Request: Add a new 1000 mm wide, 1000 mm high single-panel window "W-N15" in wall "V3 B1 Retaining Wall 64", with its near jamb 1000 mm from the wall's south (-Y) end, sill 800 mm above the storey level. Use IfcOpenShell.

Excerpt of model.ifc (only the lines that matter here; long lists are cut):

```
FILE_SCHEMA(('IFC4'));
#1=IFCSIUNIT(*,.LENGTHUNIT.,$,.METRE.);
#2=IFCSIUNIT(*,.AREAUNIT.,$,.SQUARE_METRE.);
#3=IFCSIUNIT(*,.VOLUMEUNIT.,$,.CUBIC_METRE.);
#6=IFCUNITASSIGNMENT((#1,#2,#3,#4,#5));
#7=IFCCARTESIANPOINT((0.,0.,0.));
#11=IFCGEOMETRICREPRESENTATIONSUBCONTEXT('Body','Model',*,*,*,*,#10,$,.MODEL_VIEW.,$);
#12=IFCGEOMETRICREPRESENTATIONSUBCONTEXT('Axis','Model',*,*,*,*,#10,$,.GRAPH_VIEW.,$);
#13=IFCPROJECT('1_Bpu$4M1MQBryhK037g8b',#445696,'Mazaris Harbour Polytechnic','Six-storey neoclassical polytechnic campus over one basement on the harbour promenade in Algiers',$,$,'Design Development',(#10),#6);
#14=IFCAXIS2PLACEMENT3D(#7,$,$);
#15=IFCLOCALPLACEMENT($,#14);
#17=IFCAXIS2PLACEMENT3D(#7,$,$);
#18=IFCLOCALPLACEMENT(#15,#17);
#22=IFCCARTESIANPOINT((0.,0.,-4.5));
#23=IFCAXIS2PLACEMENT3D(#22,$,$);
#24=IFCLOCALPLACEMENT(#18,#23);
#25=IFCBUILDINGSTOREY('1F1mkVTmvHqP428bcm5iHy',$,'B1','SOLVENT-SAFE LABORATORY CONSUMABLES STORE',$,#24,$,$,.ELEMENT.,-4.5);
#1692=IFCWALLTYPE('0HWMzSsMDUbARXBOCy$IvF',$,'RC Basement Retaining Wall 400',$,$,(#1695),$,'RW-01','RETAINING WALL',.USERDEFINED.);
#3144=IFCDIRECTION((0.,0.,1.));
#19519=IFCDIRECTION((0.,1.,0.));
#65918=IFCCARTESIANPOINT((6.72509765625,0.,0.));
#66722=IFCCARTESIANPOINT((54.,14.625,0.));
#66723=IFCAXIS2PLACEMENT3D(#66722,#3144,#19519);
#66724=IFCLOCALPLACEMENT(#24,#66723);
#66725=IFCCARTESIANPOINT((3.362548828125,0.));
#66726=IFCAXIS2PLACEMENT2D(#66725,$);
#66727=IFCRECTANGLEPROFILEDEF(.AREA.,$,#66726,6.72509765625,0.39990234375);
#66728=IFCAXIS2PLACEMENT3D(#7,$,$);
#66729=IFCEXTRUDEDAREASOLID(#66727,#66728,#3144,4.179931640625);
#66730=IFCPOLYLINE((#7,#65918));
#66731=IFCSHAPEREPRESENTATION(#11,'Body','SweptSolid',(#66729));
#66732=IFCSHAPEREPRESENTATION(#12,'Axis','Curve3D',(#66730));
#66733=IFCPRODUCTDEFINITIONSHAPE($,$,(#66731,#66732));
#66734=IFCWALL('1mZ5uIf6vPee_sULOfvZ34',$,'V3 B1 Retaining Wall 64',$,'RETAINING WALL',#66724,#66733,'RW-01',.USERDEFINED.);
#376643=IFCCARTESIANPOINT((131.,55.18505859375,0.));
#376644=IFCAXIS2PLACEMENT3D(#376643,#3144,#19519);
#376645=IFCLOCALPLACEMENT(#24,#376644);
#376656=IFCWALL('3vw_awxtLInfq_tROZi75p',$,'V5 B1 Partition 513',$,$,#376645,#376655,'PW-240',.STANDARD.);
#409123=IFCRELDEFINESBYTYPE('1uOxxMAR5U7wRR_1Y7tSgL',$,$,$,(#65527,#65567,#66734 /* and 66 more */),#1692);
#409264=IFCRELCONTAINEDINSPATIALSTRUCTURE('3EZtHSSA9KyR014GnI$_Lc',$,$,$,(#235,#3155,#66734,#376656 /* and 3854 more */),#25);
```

```python
import numpy as np
import ifcopenshell
import ifcopenshell.api.feature
import ifcopenshell.api.geometry
import ifcopenshell.api.root
import ifcopenshell.api.spatial
import ifcopenshell.geom
import ifcopenshell.util.element
import ifcopenshell.util.placement
import ifcopenshell.util.representation
import ifcopenshell.util.shape
import ifcopenshell.util.unit

model = ifcopenshell.open("model.ifc")
unit_scale = ifcopenshell.util.unit.calculate_unit_scale(model)
settings = ifcopenshell.geom.settings()


def volume(element):
    """Net volume in cubic metres, openings subtracted."""
    shape = ifcopenshell.geom.create_shape(settings, element)
    return ifcopenshell.util.shape.get_volume(shape.geometry)


wall = model.by_guid("1mZ5uIf6vPee_sULOfvZ34")
storey = ifcopenshell.util.element.get_container(wall, ifc_class="IfcBuildingStorey")
context = ifcopenshell.util.representation.get_context(model, "Model", "Body", "MODEL_VIEW")
before = volume(wall)

width, height, from_end, sill = 1, 1, 1, 0.8  # metres

# The wall runs along its own X axis, and the end named is its -X end.
wall_shape = ifcopenshell.geom.create_shape(settings, wall)
x, y, z = ifcopenshell.util.shape.get_vertices(wall_shape.geometry).T
start = x.min() + from_end
face, thickness = float(y.min()), float(y.max() - y.min())
wall_matrix = ifcopenshell.util.placement.get_local_placement(wall.ObjectPlacement)
level = ifcopenshell.util.placement.get_local_placement(storey.ObjectPlacement)[2, 3]


def in_wall(x, y):
    """Placement at x, y metres in the wall's axes, at sill height."""
    matrix = wall_matrix.copy()
    matrix[:, 3] = wall_matrix @ np.array([x / unit_scale, y / unit_scale, 0.0, 1.0])
    matrix[2, 3] = level + sill / unit_scale
    return matrix


# Opening: a box that overshoots both wall faces by 50 mm.
opening = ifcopenshell.api.root.create_entity(model, ifc_class="IfcOpeningElement", predefined_type="OPENING")
box = ifcopenshell.api.geometry.add_wall_representation(
    model, context=context, length=width, height=height, thickness=thickness + 0.1
)
ifcopenshell.api.geometry.assign_representation(model, product=opening, representation=box)
ifcopenshell.api.geometry.edit_object_placement(model, product=opening, matrix=in_wall(start, face - 0.05), is_si=False)
ifcopenshell.api.feature.add_feature(model, feature=opening, element=wall)

window = ifcopenshell.api.root.create_entity(model, ifc_class="IfcWindow", name="W-N15", predefined_type="WINDOW")
window.OverallWidth, window.OverallHeight = width / unit_scale, height / unit_scale
window.PartitioningType = "SINGLE_PANEL"
body = ifcopenshell.api.geometry.add_window_representation(
    model,
    context=context,
    overall_width=window.OverallWidth,
    overall_height=window.OverallHeight,
    partition_type="SINGLE_PANEL",
)
ifcopenshell.api.geometry.assign_representation(model, product=window, representation=body)
ifcopenshell.api.spatial.assign_container(model, products=[window], relating_structure=storey)
ifcopenshell.api.feature.add_filling(model, opening=opening, element=window)

# Centre the window in the wall's thickness.
ifcopenshell.api.geometry.edit_object_placement(model, product=window, matrix=in_wall(start, face), is_si=False)
window_shape = ifcopenshell.geom.create_shape(settings, window)
depth = ifcopenshell.util.shape.get_vertices(window_shape.geometry)[:, 1]
offset = face + thickness / 2 - (depth.min() + depth.max()) / 2
ifcopenshell.api.geometry.edit_object_placement(model, product=window, matrix=in_wall(start, offset), is_si=False)

after = volume(wall)

print(f"wall volume {before:.3f} -> {after:.3f} m3")

model.write("model_v2.ifc")
```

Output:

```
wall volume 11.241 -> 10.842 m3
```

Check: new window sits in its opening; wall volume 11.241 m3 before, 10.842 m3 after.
